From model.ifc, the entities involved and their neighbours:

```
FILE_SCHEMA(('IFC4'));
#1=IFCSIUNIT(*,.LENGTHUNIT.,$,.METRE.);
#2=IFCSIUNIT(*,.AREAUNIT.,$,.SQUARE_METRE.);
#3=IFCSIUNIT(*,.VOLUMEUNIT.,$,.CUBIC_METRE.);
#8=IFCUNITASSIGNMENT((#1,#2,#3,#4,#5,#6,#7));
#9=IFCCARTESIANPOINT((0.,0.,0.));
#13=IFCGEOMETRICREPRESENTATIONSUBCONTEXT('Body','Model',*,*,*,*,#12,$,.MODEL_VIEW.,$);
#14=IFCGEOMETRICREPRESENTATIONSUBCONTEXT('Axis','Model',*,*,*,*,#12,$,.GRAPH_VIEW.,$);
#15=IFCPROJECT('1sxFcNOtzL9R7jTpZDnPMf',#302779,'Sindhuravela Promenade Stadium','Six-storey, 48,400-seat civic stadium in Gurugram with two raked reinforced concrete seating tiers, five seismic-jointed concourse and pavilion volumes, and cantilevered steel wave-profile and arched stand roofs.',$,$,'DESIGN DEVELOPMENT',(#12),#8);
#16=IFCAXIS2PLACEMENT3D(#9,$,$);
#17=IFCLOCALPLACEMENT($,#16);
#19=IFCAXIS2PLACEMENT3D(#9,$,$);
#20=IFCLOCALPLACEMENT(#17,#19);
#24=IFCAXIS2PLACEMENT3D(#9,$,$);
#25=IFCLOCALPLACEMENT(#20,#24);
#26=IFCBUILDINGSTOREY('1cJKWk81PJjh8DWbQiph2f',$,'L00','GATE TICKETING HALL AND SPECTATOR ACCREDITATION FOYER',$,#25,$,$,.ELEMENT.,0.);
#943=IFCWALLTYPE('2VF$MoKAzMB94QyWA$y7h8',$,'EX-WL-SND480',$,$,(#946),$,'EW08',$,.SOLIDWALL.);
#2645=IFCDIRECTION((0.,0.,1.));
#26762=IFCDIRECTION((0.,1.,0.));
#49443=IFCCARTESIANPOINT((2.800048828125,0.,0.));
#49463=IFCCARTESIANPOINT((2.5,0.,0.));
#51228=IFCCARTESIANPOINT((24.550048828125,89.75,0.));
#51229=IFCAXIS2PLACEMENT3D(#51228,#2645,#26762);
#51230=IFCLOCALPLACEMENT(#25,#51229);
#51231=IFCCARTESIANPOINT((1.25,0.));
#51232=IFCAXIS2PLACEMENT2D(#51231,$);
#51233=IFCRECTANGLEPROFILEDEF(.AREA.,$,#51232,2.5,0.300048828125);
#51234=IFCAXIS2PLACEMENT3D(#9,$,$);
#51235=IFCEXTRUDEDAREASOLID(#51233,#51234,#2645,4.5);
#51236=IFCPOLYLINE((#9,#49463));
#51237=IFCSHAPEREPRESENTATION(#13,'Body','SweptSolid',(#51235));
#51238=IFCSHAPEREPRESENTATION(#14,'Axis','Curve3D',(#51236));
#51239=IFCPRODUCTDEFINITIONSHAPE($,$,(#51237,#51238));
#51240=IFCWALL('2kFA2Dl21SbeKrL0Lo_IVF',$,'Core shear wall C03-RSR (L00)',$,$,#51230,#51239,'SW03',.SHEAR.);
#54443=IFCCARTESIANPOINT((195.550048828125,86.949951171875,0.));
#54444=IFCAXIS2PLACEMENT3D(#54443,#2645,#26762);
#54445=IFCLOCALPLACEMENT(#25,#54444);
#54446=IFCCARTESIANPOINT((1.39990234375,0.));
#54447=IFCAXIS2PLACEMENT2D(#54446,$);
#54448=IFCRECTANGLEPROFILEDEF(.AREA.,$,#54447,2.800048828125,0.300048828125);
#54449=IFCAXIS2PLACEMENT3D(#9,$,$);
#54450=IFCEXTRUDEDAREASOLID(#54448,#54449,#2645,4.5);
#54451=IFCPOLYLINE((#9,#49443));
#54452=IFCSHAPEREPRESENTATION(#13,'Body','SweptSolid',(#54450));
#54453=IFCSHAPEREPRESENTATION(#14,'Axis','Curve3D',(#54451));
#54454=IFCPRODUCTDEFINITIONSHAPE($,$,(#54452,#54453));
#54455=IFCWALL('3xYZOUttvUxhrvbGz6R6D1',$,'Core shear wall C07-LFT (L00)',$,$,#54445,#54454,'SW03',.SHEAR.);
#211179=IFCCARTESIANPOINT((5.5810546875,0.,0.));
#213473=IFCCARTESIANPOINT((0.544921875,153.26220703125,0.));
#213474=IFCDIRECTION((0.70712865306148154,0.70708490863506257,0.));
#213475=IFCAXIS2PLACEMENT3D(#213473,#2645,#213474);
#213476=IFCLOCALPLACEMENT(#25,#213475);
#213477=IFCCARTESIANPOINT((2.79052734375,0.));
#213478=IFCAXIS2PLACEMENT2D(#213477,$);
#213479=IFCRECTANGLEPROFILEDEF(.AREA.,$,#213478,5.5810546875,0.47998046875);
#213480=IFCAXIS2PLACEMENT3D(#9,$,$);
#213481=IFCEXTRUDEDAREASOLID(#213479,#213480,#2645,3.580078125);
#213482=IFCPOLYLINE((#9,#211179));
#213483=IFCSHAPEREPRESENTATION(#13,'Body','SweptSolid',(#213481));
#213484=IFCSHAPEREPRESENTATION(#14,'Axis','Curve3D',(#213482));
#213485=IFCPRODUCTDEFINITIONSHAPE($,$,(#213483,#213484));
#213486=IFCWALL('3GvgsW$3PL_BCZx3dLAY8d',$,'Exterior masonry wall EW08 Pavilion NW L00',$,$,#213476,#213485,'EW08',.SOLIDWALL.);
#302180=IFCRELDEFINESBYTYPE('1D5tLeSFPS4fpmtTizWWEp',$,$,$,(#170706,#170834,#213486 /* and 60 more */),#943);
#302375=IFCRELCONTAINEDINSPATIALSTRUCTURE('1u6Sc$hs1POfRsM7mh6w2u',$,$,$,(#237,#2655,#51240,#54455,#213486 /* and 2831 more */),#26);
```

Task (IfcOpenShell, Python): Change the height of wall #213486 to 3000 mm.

```python
import ifcopenshell
import ifcopenshell.geom
import ifcopenshell.util.representation
import ifcopenshell.util.shape
import ifcopenshell.util.unit

model = ifcopenshell.open("model.ifc")
unit_scale = ifcopenshell.util.unit.calculate_unit_scale(model)
settings = ifcopenshell.geom.settings()


def volume(element):
    """Net volume in cubic metres, openings subtracted."""
    shape = ifcopenshell.geom.create_shape(settings, element)
    return ifcopenshell.util.shape.get_volume(shape.geometry)


wall = model.by_id(213486)
before = volume(wall)

body = ifcopenshell.util.representation.get_representation(wall, "Model", "Body")
solid = body.Items[0]
old_height = solid.Depth
solid.Depth = 3 / unit_scale
after = volume(wall)

print(f"height {old_height:g} -> {solid.Depth:g}, volume {before:.3f} -> {after:.3f} m3")

model.write("model_rev.ifc")
```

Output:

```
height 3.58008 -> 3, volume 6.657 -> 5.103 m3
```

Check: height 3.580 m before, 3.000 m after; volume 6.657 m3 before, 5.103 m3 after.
